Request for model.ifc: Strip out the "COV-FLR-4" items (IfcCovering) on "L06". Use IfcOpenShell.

First a look at what the model holds.

```python
import ifcopenshell
import ifcopenshell.util.element

model = ifcopenshell.open("model.ifc")
print(model.schema)
storey = next(s for s in model.by_type("IfcBuildingStorey") if s.Name == "L06")
coverings = [e for e in ifcopenshell.util.element.get_decomposition(storey) if e.is_a("IfcCovering")]
seen = {}
for e in coverings:
    element_type = ifcopenshell.util.element.get_type(e)
    name = element_type.Name if element_type not in (None, e) else None
    seen[name] = seen.get(name, 0) + 1
for name, count in sorted(seen.items(), key=str):
    print(count, "x", name)
```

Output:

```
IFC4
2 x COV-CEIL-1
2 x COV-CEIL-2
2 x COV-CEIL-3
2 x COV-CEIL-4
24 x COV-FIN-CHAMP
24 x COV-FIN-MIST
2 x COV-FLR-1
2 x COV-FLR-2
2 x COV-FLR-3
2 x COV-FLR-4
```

```python
import ifcopenshell
import ifcopenshell.api.root
import ifcopenshell.util.element

model = ifcopenshell.open("model.ifc")

storey = next(s for s in model.by_type("IfcBuildingStorey") if s.Name == "L06")
coverings = [e for e in ifcopenshell.util.element.get_decomposition(storey) if e.is_a("IfcCovering")]
targets = [e for e in coverings if (t := ifcopenshell.util.element.get_type(e)) not in (None, e) and t.Name == "COV-FLR-4"]

for e in targets:
    ifcopenshell.api.root.remove_product(model, product=e)
print(len(targets), "removed")

model.write("model_v2.ifc")
```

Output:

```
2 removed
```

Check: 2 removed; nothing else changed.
